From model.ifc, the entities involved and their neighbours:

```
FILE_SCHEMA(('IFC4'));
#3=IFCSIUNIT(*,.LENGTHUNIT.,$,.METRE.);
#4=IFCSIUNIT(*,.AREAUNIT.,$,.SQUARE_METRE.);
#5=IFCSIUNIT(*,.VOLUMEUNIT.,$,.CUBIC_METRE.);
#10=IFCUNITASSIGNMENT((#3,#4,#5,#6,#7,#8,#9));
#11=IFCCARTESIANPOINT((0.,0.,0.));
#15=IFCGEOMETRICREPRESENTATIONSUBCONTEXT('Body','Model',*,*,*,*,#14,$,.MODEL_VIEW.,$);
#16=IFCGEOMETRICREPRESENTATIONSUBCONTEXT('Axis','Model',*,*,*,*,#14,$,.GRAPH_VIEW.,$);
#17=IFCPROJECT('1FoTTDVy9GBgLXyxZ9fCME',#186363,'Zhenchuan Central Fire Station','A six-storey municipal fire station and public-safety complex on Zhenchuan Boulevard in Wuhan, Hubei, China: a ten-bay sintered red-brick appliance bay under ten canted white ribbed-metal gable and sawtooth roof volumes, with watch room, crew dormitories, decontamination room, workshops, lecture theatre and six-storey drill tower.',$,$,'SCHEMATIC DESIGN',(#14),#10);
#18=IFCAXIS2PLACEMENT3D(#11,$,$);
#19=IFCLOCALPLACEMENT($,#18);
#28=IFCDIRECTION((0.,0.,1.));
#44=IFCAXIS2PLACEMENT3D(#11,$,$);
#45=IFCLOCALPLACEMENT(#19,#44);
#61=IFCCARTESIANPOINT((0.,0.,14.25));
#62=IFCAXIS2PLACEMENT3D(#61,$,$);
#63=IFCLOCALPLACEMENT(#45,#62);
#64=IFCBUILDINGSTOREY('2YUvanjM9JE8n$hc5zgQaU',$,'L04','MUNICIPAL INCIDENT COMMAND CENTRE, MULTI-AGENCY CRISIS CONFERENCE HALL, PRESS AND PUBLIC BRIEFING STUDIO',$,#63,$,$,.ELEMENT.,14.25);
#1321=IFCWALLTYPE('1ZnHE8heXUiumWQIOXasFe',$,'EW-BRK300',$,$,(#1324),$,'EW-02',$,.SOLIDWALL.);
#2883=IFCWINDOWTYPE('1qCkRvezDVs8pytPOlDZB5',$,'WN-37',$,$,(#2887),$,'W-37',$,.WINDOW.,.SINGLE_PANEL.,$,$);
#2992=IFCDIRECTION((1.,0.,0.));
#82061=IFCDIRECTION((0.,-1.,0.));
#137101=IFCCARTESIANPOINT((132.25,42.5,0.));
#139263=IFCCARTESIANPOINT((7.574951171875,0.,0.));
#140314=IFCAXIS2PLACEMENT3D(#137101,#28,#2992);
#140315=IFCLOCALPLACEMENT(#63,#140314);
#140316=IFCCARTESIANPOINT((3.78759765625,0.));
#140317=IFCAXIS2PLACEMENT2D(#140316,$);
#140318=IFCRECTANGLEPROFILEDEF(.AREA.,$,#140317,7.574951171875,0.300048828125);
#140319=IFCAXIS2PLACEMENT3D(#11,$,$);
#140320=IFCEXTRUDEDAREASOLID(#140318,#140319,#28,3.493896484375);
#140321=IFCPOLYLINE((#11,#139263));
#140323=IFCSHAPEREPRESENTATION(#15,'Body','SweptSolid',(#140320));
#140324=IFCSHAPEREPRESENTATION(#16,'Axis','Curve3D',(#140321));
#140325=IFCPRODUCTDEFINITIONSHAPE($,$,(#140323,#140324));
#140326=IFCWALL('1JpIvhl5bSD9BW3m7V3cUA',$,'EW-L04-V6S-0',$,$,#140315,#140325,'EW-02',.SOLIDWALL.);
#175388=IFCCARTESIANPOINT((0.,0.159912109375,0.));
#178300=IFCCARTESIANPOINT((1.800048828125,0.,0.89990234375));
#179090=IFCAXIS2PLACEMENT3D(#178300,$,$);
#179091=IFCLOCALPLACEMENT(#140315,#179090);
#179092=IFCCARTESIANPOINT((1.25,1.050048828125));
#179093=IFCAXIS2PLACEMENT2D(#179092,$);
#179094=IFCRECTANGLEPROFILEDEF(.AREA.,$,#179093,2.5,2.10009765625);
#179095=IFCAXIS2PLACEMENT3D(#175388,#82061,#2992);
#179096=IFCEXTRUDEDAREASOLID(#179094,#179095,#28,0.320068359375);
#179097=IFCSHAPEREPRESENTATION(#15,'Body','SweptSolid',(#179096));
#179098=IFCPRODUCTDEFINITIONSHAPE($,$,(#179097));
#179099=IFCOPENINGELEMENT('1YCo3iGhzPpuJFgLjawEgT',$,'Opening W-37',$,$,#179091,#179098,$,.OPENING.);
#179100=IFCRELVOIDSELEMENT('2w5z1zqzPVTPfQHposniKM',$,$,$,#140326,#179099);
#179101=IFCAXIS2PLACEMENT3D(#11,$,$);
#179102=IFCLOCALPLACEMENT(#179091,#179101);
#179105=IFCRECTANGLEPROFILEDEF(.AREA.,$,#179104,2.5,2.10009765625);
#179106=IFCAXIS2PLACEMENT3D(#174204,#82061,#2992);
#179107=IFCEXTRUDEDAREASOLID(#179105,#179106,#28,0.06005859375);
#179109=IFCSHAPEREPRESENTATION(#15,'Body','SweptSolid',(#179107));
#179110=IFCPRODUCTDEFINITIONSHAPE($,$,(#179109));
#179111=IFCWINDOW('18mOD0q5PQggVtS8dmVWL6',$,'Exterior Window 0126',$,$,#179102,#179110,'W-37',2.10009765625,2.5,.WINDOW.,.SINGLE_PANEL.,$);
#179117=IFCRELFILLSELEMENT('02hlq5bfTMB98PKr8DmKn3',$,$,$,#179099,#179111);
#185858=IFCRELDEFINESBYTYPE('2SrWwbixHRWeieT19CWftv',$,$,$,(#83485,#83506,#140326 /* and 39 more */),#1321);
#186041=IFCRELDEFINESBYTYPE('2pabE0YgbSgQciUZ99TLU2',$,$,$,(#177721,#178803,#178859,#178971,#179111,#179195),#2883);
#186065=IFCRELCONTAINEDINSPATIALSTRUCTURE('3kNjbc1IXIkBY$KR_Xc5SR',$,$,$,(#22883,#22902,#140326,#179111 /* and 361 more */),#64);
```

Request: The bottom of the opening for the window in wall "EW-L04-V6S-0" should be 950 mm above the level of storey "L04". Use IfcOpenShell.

```python
import numpy as np
import ifcopenshell
import ifcopenshell.api.geometry
import ifcopenshell.geom
import ifcopenshell.util.element
import ifcopenshell.util.placement
import ifcopenshell.util.shape
import ifcopenshell.util.unit

model = ifcopenshell.open("model.ifc")
unit_scale = ifcopenshell.util.unit.calculate_unit_scale(model)

window = model.by_guid("18mOD0q5PQggVtS8dmVWL6")
opening = window.FillsVoids[0].RelatingOpeningElement
storey = ifcopenshell.util.element.get_container(window, ifc_class="IfcBuildingStorey")
level = ifcopenshell.util.placement.get_local_placement(storey.ObjectPlacement)[2, 3]

# The opening's origin need not be at the sill, so measure its lowest point.
shape = ifcopenshell.geom.create_shape(ifcopenshell.geom.settings(), opening)
bottom = ifcopenshell.util.shape.get_shape_bottom_elevation(shape, shape.geometry) / unit_scale
dz = level + 0.95 / unit_scale - bottom

shift = np.array([0.0, 0.0, dz])
# The window is placed relative to its opening, so it follows when the opening moves.
matrix = ifcopenshell.util.placement.get_local_placement(opening.ObjectPlacement)
matrix[:3, 3] += shift
ifcopenshell.api.geometry.edit_object_placement(
    model, product=opening, matrix=matrix, is_si=False, should_transform_children=True
)

print(f"moved by {dz * unit_scale:+.3f} m")

model.write("model_edited.ifc")
```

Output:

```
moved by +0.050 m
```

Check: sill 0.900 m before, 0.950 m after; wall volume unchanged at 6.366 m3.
